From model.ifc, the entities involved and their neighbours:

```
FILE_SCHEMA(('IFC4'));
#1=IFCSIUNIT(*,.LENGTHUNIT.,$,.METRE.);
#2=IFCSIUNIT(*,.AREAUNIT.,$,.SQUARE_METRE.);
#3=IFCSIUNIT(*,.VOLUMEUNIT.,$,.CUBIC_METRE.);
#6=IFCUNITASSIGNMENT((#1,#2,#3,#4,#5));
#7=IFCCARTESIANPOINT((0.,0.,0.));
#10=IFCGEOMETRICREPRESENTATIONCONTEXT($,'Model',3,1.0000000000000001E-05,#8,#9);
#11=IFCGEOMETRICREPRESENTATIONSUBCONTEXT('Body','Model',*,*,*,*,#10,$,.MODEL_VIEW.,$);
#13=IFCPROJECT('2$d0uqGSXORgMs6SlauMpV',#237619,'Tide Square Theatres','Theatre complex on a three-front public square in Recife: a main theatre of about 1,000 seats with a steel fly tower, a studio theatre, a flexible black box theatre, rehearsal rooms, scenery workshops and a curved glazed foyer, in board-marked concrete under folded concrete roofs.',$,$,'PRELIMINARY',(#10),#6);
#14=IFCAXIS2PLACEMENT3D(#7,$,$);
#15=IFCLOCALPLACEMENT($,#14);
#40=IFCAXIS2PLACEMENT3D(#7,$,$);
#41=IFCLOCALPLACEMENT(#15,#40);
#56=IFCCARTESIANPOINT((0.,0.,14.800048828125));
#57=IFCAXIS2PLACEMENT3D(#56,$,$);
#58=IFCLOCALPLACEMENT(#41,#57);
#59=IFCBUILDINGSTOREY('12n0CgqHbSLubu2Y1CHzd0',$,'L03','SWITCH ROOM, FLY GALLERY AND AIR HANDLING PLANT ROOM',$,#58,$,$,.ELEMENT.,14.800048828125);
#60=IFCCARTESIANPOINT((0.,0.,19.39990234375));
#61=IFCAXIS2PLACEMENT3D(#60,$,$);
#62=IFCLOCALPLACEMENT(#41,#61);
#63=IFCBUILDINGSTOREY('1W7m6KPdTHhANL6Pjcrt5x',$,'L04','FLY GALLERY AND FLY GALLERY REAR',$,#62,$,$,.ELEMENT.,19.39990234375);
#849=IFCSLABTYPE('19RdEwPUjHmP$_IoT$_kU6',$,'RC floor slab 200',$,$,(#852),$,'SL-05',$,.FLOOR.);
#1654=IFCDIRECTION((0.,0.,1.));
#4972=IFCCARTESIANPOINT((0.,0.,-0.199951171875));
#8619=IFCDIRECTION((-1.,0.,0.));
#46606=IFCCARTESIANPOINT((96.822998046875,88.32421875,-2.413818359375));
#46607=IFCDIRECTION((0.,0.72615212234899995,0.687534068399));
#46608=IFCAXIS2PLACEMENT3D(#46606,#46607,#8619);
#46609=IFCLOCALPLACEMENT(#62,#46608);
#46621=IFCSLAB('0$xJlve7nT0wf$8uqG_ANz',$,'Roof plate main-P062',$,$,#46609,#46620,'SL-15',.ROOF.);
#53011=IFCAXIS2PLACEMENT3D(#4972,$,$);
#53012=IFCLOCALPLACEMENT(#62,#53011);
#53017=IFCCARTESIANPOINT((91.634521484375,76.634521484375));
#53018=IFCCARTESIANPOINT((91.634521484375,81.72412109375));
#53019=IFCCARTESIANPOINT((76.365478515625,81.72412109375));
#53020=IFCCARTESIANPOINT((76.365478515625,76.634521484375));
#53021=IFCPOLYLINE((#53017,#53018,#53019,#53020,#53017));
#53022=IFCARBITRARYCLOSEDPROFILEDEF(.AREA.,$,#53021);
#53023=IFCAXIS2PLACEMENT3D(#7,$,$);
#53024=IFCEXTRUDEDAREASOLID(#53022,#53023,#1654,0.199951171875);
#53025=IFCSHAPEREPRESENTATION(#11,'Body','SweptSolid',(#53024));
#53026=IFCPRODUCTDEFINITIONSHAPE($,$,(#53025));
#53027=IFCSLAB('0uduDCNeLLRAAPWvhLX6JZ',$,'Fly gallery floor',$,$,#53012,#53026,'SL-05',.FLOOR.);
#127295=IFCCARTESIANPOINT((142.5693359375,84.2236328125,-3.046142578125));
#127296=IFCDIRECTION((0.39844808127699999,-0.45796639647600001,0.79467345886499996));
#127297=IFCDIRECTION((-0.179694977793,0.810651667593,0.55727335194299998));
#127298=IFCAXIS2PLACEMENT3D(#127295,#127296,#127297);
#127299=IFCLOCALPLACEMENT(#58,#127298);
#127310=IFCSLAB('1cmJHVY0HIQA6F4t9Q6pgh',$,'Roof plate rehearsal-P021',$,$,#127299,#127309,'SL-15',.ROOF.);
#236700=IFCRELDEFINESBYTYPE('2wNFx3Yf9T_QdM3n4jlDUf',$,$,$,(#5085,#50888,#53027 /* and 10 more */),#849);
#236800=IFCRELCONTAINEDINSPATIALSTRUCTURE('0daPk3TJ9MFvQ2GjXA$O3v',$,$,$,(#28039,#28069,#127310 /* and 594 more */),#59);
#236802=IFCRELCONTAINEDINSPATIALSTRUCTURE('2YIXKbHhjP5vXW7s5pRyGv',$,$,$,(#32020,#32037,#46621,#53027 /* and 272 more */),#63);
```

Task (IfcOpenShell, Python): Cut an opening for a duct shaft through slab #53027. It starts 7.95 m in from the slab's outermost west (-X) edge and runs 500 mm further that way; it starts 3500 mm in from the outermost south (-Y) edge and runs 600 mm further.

```python
import numpy as np
import ifcopenshell
import ifcopenshell.api.feature
import ifcopenshell.api.geometry
import ifcopenshell.api.root
import ifcopenshell.geom
import ifcopenshell.util.placement
import ifcopenshell.util.representation
import ifcopenshell.util.shape
import ifcopenshell.util.unit

model = ifcopenshell.open("model.ifc")
unit_scale = ifcopenshell.util.unit.calculate_unit_scale(model)
settings = ifcopenshell.geom.settings()


def volume(element):
    """Net volume in cubic metres, openings subtracted."""
    shape = ifcopenshell.geom.create_shape(settings, element)
    return ifcopenshell.util.shape.get_volume(shape.geometry)


slab = model.by_guid("0uduDCNeLLRAAPWvhLX6JZ")
before = volume(slab)

# Extent in the slab's own axes, in metres. The edges named are its -X and -Y sides.
slab_shape = ifcopenshell.geom.create_shape(settings, slab)
vertices = ifcopenshell.util.shape.get_vertices(slab_shape.geometry)
x_min, y_min, bottom = vertices.min(axis=0)
top = vertices[:, 2].max()

opening = ifcopenshell.api.root.create_entity(model, ifc_class="IfcOpeningElement", name="Duct shaft opening", predefined_type="OPENING")
context = ifcopenshell.util.representation.get_context(model, "Model", "Body", "MODEL_VIEW")
width, depth = 0.5, 0.6
outline = [(0.0, 0.0), (width, 0.0), (width, depth), (0.0, depth), (0.0, 0.0)]
# Overshoot both faces by 50 mm so the cut is clean.
shape = ifcopenshell.api.geometry.add_slab_representation(
    model, context=context, depth=top - bottom + 0.1, polyline=outline
)
ifcopenshell.api.geometry.assign_representation(model, product=opening, representation=shape)

matrix = ifcopenshell.util.placement.get_local_placement(slab.ObjectPlacement)
matrix[:, 3] = matrix @ np.append(np.array([x_min + 7.95, y_min + 3.5, bottom - 0.05]) / unit_scale, 1.0)
ifcopenshell.api.geometry.edit_object_placement(model, product=opening, matrix=matrix, is_si=False)
ifcopenshell.api.feature.add_feature(model, feature=opening, element=slab)

after = volume(slab)

print(f"slab volume {before:.3f} -> {after:.3f} m3")

model.write("model_v2.ifc")
```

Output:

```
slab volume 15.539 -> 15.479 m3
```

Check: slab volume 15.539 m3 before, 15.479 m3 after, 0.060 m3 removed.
